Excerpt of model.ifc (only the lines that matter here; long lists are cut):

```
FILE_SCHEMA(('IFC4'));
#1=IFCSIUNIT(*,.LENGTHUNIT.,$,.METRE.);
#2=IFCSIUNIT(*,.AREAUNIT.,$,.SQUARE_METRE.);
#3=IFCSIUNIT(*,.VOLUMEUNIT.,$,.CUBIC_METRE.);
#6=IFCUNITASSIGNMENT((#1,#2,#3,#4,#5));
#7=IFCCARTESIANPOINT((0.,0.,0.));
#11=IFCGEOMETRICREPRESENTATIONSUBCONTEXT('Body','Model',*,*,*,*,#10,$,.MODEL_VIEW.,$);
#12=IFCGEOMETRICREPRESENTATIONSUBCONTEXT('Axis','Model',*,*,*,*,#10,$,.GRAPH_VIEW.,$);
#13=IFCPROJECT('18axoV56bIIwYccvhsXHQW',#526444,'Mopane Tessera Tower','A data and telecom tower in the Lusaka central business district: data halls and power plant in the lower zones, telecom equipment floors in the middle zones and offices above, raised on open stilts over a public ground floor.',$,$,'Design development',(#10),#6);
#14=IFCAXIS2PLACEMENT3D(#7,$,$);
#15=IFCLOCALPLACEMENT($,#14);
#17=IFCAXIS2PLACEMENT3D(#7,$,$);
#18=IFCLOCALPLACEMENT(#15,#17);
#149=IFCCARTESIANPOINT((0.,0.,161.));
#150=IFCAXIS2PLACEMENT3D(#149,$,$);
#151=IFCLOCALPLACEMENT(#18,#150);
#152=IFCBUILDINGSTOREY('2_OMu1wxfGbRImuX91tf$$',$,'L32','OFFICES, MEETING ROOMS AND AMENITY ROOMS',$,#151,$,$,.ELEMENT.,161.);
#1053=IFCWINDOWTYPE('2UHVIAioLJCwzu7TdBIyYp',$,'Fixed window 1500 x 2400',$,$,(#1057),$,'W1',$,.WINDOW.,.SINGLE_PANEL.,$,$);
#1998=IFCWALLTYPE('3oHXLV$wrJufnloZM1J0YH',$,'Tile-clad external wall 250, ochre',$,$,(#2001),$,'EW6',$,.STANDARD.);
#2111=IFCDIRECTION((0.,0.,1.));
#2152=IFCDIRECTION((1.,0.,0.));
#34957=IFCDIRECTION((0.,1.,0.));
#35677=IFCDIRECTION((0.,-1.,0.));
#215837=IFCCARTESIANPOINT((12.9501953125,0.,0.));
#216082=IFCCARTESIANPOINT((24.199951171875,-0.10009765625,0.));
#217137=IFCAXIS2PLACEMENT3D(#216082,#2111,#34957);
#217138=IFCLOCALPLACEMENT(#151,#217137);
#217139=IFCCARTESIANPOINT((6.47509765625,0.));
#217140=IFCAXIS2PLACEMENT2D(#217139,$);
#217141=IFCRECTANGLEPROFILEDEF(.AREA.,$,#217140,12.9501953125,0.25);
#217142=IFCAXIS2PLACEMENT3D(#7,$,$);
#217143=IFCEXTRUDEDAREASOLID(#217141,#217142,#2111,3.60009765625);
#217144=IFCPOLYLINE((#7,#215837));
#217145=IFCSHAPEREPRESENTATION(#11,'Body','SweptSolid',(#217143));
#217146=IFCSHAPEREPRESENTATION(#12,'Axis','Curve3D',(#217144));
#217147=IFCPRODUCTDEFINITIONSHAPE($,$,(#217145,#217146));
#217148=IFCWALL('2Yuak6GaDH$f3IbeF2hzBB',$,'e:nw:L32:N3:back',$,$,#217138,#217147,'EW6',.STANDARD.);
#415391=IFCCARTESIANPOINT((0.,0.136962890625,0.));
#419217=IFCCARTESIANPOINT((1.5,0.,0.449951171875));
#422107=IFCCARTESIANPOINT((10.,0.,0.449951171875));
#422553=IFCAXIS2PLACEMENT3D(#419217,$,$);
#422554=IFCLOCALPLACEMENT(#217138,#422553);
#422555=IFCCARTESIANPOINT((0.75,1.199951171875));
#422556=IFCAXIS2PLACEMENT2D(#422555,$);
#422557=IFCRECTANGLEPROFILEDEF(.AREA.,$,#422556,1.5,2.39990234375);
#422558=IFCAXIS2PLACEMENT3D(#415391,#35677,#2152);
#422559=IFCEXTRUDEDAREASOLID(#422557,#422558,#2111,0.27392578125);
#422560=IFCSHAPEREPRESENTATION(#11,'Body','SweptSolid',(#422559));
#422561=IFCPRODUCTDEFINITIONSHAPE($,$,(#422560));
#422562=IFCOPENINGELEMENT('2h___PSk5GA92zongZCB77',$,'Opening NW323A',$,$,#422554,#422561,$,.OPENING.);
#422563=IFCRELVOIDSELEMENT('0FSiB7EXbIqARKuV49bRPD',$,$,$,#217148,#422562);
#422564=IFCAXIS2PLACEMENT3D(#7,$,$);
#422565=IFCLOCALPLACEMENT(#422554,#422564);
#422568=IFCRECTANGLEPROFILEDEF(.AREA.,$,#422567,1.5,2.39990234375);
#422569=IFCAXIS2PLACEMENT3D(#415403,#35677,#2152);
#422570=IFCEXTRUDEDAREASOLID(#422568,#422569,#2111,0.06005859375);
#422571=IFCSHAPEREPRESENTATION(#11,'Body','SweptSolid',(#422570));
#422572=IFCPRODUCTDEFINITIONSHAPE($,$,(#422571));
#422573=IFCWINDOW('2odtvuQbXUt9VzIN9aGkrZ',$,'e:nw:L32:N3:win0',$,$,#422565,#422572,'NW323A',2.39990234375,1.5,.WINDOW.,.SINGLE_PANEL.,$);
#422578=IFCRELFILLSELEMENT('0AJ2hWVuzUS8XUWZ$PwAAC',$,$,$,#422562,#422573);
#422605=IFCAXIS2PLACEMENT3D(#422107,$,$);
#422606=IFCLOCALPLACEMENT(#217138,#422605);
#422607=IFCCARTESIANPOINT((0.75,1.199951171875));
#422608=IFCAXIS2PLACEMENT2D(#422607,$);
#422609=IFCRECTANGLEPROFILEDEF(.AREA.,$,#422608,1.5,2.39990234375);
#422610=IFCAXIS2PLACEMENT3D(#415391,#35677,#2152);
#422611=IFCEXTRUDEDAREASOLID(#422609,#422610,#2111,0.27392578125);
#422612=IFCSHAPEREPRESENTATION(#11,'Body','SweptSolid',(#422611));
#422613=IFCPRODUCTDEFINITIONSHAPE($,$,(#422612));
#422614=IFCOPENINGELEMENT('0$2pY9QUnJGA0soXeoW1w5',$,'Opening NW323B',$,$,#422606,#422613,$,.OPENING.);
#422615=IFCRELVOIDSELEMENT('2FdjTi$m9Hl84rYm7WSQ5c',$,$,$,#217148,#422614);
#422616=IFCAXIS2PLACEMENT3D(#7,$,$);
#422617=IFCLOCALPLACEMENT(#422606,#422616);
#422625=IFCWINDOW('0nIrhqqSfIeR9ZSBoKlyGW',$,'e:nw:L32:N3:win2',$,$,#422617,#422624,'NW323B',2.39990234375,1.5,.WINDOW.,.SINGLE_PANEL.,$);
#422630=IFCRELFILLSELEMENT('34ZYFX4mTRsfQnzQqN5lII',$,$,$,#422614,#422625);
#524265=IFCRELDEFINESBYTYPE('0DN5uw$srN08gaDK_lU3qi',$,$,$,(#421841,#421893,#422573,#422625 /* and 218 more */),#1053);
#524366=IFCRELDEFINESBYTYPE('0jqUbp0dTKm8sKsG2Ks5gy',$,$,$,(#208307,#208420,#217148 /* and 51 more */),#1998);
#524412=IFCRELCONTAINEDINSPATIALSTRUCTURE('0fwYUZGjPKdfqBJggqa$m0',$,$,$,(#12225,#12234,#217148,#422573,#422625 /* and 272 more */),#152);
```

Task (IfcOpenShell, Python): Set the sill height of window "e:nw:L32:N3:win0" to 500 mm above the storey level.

```python
import numpy as np
import ifcopenshell
import ifcopenshell.api.geometry
import ifcopenshell.geom
import ifcopenshell.util.element
import ifcopenshell.util.placement
import ifcopenshell.util.shape
import ifcopenshell.util.unit

model = ifcopenshell.open("model.ifc")
unit_scale = ifcopenshell.util.unit.calculate_unit_scale(model)

window = model.by_guid("2odtvuQbXUt9VzIN9aGkrZ")
opening = window.FillsVoids[0].RelatingOpeningElement
storey = ifcopenshell.util.element.get_container(window, ifc_class="IfcBuildingStorey")
level = ifcopenshell.util.placement.get_local_placement(storey.ObjectPlacement)[2, 3]

# The opening's origin need not be at the sill, so measure its lowest point.
shape = ifcopenshell.geom.create_shape(ifcopenshell.geom.settings(), opening)
bottom = ifcopenshell.util.shape.get_shape_bottom_elevation(shape, shape.geometry) / unit_scale
dz = level + 0.5 / unit_scale - bottom

shift = np.array([0.0, 0.0, dz])
# The window is placed relative to its opening, so it follows when the opening moves.
matrix = ifcopenshell.util.placement.get_local_placement(opening.ObjectPlacement)
matrix[:3, 3] += shift
ifcopenshell.api.geometry.edit_object_placement(
    model, product=opening, matrix=matrix, is_si=False, should_transform_children=True
)

print(f"moved by {dz * unit_scale:+.3f} m")

model.write("model_v2.ifc")
```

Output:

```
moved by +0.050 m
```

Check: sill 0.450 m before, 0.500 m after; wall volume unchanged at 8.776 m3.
